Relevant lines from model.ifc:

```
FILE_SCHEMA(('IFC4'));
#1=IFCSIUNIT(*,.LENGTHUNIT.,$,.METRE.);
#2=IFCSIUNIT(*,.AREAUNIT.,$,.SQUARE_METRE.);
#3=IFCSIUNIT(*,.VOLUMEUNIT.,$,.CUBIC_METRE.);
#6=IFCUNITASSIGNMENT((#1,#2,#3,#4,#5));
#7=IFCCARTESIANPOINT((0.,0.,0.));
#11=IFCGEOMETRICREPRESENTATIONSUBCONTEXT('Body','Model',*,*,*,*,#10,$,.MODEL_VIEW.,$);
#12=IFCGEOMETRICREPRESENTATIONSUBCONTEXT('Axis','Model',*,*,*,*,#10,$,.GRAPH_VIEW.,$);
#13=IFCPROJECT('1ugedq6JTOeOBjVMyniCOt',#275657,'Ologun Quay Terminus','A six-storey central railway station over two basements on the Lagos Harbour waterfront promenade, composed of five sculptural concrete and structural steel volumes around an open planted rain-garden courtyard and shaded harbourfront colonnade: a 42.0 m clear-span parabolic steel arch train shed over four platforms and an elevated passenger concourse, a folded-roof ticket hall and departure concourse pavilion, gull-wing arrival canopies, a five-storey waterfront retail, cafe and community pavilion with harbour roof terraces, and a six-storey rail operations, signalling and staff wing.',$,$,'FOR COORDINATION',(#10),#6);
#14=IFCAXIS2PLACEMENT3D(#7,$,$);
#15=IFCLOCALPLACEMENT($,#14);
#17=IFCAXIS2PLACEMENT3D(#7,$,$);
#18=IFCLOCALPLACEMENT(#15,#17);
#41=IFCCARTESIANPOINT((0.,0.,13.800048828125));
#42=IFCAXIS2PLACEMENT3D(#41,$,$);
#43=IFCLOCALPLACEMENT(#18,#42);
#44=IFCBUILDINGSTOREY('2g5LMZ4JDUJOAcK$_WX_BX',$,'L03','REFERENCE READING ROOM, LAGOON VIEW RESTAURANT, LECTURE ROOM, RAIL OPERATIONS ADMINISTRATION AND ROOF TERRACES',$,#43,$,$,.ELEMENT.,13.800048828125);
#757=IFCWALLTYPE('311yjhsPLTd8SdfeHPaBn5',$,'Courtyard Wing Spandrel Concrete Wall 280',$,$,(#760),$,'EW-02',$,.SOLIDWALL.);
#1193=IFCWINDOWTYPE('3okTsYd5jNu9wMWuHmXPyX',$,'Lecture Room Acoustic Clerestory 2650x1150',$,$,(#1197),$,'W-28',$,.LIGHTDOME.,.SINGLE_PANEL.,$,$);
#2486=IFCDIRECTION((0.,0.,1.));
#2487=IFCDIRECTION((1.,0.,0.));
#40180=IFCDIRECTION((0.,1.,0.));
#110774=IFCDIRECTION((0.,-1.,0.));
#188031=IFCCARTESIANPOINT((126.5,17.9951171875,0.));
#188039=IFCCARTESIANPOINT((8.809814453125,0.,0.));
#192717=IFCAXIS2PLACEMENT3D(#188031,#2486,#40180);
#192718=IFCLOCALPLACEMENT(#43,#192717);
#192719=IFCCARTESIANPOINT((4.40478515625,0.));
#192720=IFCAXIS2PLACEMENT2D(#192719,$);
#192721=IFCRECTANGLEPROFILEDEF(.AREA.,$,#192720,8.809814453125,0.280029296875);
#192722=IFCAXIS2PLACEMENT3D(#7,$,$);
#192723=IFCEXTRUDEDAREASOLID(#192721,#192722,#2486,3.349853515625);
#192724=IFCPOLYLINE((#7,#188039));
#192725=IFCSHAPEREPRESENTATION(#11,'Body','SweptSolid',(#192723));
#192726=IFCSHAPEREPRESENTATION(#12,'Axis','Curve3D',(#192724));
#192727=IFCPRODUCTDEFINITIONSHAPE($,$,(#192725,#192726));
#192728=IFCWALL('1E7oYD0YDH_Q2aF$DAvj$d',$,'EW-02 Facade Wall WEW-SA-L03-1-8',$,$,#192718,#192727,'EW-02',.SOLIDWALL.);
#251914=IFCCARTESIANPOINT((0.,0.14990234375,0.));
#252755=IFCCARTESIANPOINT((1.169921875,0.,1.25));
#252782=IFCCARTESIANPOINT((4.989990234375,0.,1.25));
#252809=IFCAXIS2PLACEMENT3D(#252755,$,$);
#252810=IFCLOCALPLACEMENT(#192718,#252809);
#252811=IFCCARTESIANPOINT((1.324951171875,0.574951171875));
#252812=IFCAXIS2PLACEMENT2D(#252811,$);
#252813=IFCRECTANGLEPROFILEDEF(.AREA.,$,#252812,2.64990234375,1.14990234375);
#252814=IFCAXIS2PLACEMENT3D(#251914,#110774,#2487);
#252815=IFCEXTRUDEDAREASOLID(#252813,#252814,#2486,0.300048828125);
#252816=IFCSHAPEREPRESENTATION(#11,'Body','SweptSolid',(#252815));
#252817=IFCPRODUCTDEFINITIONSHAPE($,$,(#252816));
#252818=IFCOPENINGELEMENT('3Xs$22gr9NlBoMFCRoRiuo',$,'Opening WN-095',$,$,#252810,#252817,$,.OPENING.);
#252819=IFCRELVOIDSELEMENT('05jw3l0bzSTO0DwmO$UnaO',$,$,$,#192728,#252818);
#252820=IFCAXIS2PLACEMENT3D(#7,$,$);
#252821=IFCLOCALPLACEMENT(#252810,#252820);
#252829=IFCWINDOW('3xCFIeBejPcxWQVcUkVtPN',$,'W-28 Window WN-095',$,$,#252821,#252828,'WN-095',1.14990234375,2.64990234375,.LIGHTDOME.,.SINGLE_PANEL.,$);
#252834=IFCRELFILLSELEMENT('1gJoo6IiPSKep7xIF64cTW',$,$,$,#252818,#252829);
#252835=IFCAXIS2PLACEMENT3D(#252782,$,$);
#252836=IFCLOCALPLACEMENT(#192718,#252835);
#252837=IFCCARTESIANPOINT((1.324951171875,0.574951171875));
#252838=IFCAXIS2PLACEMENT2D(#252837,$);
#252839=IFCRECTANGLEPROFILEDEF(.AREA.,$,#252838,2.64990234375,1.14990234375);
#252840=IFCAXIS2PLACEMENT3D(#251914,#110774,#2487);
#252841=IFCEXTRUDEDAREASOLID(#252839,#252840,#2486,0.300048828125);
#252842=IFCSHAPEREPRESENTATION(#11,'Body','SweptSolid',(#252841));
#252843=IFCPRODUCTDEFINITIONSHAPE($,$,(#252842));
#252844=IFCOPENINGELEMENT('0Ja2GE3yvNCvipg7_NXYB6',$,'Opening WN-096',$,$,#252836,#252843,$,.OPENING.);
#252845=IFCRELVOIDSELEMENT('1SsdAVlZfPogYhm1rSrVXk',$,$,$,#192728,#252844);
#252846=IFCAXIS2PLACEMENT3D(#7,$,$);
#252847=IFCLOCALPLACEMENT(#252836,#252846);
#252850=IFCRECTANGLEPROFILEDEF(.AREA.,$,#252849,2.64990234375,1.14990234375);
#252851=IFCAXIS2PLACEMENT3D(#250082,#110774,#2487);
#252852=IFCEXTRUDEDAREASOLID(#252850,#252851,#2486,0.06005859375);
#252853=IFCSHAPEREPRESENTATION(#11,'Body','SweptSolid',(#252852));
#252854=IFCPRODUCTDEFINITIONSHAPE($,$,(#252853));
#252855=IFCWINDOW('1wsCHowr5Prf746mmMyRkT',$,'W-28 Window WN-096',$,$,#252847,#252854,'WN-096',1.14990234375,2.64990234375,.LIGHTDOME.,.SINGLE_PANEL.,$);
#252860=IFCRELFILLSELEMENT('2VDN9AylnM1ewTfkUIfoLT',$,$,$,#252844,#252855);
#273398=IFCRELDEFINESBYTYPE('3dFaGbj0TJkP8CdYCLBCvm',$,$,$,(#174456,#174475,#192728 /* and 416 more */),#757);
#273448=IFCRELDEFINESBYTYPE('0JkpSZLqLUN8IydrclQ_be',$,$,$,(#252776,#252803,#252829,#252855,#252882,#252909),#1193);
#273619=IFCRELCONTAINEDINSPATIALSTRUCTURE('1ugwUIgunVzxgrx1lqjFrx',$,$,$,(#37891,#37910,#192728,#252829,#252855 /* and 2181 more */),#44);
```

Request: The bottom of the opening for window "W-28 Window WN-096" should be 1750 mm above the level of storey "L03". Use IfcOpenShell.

```python
import numpy as np
import ifcopenshell
import ifcopenshell.api.geometry
import ifcopenshell.geom
import ifcopenshell.util.element
import ifcopenshell.util.placement
import ifcopenshell.util.shape
import ifcopenshell.util.unit

model = ifcopenshell.open("model.ifc")
unit_scale = ifcopenshell.util.unit.calculate_unit_scale(model)

window = model.by_guid("1wsCHowr5Prf746mmMyRkT")
opening = window.FillsVoids[0].RelatingOpeningElement
storey = ifcopenshell.util.element.get_container(window, ifc_class="IfcBuildingStorey")
level = ifcopenshell.util.placement.get_local_placement(storey.ObjectPlacement)[2, 3]

# The opening's origin need not be at the sill, so measure its lowest point.
shape = ifcopenshell.geom.create_shape(ifcopenshell.geom.settings(), opening)
bottom = ifcopenshell.util.shape.get_shape_bottom_elevation(shape, shape.geometry) / unit_scale
dz = level + 1.75 / unit_scale - bottom

shift = np.array([0.0, 0.0, dz])
# The window is placed relative to its opening, so it follows when the opening moves.
matrix = ifcopenshell.util.placement.get_local_placement(opening.ObjectPlacement)
matrix[:3, 3] += shift
ifcopenshell.api.geometry.edit_object_placement(
    model, product=opening, matrix=matrix, is_si=False, should_transform_children=True
)

print(f"moved by {dz * unit_scale:+.3f} m")

model.write("model_updated.ifc")
```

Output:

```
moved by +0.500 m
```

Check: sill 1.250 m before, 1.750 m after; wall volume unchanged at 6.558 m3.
